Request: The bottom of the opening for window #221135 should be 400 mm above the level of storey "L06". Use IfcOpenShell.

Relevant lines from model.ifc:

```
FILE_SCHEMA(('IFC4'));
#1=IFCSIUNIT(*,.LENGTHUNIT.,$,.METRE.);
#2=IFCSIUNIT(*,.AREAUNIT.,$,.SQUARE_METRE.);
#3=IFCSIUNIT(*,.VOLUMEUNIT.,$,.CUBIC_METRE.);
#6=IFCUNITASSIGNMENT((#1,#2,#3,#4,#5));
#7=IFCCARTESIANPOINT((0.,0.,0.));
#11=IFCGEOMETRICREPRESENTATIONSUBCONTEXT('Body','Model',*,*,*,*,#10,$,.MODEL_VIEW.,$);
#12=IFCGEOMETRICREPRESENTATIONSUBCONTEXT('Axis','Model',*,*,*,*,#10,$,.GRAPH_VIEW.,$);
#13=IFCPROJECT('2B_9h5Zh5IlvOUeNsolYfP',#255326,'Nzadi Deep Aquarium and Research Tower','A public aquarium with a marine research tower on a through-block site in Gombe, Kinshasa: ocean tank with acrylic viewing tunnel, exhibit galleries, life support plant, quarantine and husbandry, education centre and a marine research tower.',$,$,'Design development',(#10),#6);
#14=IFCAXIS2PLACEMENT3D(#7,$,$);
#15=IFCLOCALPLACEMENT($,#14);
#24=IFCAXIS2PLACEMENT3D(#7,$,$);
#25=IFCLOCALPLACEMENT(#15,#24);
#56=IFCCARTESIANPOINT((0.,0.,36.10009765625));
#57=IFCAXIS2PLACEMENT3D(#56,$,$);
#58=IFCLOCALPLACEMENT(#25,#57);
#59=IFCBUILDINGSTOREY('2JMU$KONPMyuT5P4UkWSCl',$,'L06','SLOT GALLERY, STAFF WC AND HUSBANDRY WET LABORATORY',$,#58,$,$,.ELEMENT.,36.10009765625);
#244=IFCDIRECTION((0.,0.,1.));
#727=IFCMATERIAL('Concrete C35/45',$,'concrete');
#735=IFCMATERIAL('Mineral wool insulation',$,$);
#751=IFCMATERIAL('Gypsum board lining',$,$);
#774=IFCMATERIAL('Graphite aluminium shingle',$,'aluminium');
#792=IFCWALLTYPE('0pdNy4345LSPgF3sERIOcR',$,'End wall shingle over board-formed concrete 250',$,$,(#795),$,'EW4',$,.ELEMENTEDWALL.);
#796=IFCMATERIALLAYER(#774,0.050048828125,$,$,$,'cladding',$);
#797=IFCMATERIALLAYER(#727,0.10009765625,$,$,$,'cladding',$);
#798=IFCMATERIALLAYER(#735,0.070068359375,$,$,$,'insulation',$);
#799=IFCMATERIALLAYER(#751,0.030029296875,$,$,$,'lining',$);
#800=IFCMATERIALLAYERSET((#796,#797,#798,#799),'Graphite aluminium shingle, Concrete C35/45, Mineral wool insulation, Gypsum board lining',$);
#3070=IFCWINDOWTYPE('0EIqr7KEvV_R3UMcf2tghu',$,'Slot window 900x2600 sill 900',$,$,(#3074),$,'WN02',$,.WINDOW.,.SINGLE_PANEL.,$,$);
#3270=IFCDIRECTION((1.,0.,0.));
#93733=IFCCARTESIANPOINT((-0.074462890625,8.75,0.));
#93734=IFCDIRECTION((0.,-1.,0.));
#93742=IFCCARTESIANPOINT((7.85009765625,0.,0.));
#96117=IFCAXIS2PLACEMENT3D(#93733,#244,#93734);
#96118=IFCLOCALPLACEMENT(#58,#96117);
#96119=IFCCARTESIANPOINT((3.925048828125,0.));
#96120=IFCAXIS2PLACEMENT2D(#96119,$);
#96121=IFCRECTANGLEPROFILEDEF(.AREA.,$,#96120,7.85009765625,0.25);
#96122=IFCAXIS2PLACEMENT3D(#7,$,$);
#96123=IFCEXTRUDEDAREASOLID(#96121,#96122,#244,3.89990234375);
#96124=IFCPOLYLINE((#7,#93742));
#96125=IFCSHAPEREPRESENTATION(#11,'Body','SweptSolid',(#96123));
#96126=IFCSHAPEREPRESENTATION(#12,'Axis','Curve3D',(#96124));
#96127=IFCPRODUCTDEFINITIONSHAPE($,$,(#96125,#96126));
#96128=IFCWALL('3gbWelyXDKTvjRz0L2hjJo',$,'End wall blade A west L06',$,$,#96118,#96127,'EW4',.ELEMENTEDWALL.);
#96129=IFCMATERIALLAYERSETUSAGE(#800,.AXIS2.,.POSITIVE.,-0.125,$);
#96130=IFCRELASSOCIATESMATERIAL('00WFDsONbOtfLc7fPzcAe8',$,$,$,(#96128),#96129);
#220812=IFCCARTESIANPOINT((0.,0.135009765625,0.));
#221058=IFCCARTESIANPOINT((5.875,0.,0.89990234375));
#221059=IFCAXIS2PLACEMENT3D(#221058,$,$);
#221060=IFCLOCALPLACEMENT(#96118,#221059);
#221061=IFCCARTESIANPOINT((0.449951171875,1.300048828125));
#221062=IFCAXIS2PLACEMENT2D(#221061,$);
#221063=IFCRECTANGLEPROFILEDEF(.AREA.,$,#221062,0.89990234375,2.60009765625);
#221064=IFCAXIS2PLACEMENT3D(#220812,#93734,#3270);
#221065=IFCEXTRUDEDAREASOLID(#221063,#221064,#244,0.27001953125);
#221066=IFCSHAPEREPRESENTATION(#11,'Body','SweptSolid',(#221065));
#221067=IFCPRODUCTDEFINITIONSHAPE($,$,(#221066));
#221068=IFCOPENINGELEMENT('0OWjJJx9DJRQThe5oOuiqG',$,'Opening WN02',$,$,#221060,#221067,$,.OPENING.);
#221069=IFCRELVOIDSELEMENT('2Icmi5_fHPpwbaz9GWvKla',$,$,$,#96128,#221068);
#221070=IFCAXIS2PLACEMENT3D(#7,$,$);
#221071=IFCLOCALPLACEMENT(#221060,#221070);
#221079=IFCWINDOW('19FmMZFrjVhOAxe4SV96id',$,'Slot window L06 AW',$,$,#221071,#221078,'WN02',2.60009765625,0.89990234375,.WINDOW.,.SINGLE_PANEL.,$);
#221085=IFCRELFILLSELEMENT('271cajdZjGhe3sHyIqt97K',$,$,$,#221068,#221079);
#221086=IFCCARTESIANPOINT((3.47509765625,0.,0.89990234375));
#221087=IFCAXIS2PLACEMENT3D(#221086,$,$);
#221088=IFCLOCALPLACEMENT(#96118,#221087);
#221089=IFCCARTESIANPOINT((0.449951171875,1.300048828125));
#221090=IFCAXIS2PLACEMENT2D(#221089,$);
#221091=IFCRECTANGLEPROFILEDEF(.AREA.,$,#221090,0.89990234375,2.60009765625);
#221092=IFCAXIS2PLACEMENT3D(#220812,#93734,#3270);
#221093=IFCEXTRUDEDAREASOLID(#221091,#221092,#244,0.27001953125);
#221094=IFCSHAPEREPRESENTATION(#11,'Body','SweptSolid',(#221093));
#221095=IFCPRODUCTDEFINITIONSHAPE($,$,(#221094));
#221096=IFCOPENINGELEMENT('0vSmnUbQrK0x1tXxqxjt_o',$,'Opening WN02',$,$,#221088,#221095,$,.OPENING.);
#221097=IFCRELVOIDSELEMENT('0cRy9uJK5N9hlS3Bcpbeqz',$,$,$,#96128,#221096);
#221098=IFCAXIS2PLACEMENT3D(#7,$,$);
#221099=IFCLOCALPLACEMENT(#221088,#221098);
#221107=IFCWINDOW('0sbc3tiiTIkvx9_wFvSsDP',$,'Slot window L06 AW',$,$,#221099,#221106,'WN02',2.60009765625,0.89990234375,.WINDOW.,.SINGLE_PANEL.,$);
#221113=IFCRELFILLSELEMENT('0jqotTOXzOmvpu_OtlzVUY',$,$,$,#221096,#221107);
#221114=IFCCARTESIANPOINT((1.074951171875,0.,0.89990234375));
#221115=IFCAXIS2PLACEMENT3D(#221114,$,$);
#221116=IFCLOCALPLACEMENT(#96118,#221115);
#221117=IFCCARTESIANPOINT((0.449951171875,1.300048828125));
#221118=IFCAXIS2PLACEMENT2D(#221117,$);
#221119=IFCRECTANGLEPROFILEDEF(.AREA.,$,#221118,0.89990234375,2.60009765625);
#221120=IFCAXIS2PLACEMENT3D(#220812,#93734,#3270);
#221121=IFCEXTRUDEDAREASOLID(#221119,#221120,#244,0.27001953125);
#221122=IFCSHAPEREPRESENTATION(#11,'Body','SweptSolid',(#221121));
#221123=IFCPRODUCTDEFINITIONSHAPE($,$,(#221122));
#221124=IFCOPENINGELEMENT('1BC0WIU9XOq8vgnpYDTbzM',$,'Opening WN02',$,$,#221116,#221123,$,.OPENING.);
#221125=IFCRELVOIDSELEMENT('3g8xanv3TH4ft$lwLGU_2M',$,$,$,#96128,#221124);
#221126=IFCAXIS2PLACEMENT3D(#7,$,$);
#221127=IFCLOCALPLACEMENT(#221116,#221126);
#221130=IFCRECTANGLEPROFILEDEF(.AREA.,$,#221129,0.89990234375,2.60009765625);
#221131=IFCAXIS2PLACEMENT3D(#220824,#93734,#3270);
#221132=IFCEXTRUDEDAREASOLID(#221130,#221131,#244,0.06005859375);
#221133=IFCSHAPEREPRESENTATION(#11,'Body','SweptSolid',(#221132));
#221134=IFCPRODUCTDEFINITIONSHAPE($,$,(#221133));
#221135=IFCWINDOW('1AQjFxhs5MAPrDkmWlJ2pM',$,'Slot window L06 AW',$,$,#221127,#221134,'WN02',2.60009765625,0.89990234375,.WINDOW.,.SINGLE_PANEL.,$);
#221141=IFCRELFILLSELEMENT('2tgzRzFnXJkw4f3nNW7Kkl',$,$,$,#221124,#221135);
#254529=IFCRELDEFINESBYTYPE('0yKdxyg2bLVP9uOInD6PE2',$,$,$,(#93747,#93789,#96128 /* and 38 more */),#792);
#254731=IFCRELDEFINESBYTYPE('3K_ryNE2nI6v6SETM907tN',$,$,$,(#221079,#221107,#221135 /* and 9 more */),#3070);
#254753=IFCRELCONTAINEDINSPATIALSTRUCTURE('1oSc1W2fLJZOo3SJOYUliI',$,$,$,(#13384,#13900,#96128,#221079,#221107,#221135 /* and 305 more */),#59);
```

```python
import numpy as np
import ifcopenshell
import ifcopenshell.api.geometry
import ifcopenshell.geom
import ifcopenshell.util.element
import ifcopenshell.util.placement
import ifcopenshell.util.shape
import ifcopenshell.util.unit

model = ifcopenshell.open("model.ifc")
unit_scale = ifcopenshell.util.unit.calculate_unit_scale(model)

window = model.by_guid("1AQjFxhs5MAPrDkmWlJ2pM")
opening = window.FillsVoids[0].RelatingOpeningElement
storey = ifcopenshell.util.element.get_container(window, ifc_class="IfcBuildingStorey")
level = ifcopenshell.util.placement.get_local_placement(storey.ObjectPlacement)[2, 3]

# The opening's origin need not be at the sill, so measure its lowest point.
shape = ifcopenshell.geom.create_shape(ifcopenshell.geom.settings(), opening)
bottom = ifcopenshell.util.shape.get_shape_bottom_elevation(shape, shape.geometry) / unit_scale
dz = level + 0.4 / unit_scale - bottom

shift = np.array([0.0, 0.0, dz])
# The window is placed relative to its opening, so it follows when the opening moves.
matrix = ifcopenshell.util.placement.get_local_placement(opening.ObjectPlacement)
matrix[:3, 3] += shift
ifcopenshell.api.geometry.edit_object_placement(
    model, product=opening, matrix=matrix, is_si=False, should_transform_children=True
)

print(f"moved by {dz * unit_scale:+.3f} m")

model.write("model_edited.ifc")
```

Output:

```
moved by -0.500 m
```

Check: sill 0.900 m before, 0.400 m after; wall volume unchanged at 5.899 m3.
